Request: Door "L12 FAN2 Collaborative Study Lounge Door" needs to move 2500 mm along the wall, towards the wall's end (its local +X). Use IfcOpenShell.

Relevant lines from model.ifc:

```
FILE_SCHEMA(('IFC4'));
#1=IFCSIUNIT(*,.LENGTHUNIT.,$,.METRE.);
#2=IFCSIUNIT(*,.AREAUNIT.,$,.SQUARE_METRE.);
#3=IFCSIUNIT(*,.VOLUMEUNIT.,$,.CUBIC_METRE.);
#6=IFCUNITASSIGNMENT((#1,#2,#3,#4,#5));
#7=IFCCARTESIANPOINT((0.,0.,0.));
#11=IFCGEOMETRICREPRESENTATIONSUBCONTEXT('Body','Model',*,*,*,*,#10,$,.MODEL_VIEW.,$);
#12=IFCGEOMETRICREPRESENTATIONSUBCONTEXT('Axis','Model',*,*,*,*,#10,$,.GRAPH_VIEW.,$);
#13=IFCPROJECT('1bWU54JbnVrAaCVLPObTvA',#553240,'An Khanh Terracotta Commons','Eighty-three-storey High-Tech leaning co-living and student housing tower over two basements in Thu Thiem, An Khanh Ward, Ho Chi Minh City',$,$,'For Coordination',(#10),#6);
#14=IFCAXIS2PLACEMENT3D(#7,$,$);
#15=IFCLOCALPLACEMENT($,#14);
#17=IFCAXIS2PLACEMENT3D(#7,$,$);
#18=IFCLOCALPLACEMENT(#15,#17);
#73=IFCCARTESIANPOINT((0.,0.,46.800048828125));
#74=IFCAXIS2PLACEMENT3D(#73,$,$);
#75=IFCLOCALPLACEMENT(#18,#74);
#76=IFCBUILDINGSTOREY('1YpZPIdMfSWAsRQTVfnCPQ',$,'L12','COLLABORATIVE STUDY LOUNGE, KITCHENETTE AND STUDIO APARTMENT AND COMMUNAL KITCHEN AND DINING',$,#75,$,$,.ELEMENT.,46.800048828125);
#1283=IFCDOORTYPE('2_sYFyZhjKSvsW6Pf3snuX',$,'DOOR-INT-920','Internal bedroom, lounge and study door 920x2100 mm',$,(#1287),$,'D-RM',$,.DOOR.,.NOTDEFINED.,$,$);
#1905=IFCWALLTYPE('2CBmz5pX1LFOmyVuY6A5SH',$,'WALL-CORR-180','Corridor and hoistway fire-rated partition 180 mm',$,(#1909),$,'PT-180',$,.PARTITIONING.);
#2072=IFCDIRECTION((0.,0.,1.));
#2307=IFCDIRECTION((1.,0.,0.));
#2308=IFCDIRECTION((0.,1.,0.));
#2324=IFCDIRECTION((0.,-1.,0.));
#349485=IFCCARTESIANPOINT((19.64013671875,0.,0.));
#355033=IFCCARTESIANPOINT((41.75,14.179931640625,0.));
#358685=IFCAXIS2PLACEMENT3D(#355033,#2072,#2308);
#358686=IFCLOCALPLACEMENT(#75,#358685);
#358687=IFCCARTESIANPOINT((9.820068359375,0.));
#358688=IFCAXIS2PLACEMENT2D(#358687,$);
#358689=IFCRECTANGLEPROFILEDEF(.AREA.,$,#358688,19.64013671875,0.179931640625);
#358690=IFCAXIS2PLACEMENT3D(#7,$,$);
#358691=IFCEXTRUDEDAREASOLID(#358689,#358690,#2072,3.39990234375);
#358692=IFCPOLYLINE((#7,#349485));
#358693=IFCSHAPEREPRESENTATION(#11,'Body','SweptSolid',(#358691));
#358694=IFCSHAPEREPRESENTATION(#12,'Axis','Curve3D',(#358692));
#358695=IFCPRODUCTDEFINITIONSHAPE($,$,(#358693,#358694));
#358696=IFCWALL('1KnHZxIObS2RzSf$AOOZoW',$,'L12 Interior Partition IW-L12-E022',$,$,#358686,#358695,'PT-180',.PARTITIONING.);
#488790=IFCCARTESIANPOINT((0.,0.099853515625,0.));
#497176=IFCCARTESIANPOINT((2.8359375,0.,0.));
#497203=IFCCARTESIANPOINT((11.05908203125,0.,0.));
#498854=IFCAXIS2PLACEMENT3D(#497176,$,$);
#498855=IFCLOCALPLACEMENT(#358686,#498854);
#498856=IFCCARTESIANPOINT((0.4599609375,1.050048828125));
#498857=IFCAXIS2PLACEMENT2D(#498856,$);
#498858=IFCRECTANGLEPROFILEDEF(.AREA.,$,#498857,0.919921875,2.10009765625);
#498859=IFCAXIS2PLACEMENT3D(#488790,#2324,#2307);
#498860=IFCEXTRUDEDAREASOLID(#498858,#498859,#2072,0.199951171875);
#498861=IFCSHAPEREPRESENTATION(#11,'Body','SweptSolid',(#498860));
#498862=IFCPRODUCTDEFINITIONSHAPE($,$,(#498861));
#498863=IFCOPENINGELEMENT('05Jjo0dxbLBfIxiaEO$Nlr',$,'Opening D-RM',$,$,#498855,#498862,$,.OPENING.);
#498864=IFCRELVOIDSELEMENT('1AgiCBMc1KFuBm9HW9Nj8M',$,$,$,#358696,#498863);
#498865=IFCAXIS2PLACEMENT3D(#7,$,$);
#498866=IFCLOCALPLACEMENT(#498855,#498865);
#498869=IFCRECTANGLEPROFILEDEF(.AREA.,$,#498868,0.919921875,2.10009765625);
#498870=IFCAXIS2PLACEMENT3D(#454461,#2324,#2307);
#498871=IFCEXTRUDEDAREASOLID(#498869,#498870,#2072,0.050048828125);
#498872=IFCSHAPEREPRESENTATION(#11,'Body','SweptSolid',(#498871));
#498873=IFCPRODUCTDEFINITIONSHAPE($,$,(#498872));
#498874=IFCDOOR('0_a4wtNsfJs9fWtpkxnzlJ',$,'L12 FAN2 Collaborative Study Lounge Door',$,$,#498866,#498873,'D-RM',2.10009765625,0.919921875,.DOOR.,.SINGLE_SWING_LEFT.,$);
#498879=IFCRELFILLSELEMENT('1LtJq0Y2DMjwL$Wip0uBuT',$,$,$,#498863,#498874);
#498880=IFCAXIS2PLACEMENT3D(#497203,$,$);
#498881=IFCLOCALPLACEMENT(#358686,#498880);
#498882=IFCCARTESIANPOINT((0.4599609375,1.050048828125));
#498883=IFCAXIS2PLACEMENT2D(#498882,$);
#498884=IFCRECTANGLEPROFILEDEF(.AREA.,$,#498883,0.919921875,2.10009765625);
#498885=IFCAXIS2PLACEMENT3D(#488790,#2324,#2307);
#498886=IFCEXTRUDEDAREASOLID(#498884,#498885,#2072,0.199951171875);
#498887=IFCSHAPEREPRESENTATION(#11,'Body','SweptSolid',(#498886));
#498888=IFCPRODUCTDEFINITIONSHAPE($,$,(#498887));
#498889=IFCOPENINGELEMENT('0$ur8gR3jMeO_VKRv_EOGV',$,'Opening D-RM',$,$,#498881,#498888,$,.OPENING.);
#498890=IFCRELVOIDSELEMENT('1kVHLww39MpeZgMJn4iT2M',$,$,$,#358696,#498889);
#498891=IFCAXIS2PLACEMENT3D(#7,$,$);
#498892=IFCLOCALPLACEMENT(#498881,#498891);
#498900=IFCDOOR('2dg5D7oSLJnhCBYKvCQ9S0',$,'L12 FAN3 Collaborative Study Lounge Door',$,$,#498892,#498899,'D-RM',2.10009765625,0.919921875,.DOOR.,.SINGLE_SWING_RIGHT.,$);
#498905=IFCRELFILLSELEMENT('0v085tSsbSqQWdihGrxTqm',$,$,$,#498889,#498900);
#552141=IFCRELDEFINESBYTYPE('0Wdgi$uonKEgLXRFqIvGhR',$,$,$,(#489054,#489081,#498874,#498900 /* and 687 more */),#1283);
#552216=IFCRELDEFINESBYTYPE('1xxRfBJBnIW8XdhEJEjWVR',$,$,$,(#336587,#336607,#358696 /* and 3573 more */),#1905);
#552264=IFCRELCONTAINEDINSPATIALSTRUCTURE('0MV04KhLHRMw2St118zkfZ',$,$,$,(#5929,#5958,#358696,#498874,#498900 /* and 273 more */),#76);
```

```python
import ifcopenshell
import ifcopenshell.api.geometry
import ifcopenshell.util.placement
import ifcopenshell.util.unit

model = ifcopenshell.open("model.ifc")
unit_scale = ifcopenshell.util.unit.calculate_unit_scale(model)

door = model.by_guid("0_a4wtNsfJs9fWtpkxnzlJ")
opening = door.FillsVoids[0].RelatingOpeningElement
wall = opening.VoidsElements[0].RelatingBuildingElement

wall_matrix = ifcopenshell.util.placement.get_local_placement(wall.ObjectPlacement)
shift = wall_matrix[:3, 0] * 2.5 / unit_scale
before = ifcopenshell.util.placement.get_local_placement(door.ObjectPlacement)[:3, 3].copy()

# The door is placed relative to its opening, so it follows when the opening moves.
matrix = ifcopenshell.util.placement.get_local_placement(opening.ObjectPlacement)
matrix[:3, 3] += shift
ifcopenshell.api.geometry.edit_object_placement(
    model, product=opening, matrix=matrix, is_si=False, should_transform_children=True
)

after = ifcopenshell.util.placement.get_local_placement(door.ObjectPlacement)[:3, 3]
print("door moved by", (after - before).round(3) + 0.0)

model.write("model_edited.ifc")
```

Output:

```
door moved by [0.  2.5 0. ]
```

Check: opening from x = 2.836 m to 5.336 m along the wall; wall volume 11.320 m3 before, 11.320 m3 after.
